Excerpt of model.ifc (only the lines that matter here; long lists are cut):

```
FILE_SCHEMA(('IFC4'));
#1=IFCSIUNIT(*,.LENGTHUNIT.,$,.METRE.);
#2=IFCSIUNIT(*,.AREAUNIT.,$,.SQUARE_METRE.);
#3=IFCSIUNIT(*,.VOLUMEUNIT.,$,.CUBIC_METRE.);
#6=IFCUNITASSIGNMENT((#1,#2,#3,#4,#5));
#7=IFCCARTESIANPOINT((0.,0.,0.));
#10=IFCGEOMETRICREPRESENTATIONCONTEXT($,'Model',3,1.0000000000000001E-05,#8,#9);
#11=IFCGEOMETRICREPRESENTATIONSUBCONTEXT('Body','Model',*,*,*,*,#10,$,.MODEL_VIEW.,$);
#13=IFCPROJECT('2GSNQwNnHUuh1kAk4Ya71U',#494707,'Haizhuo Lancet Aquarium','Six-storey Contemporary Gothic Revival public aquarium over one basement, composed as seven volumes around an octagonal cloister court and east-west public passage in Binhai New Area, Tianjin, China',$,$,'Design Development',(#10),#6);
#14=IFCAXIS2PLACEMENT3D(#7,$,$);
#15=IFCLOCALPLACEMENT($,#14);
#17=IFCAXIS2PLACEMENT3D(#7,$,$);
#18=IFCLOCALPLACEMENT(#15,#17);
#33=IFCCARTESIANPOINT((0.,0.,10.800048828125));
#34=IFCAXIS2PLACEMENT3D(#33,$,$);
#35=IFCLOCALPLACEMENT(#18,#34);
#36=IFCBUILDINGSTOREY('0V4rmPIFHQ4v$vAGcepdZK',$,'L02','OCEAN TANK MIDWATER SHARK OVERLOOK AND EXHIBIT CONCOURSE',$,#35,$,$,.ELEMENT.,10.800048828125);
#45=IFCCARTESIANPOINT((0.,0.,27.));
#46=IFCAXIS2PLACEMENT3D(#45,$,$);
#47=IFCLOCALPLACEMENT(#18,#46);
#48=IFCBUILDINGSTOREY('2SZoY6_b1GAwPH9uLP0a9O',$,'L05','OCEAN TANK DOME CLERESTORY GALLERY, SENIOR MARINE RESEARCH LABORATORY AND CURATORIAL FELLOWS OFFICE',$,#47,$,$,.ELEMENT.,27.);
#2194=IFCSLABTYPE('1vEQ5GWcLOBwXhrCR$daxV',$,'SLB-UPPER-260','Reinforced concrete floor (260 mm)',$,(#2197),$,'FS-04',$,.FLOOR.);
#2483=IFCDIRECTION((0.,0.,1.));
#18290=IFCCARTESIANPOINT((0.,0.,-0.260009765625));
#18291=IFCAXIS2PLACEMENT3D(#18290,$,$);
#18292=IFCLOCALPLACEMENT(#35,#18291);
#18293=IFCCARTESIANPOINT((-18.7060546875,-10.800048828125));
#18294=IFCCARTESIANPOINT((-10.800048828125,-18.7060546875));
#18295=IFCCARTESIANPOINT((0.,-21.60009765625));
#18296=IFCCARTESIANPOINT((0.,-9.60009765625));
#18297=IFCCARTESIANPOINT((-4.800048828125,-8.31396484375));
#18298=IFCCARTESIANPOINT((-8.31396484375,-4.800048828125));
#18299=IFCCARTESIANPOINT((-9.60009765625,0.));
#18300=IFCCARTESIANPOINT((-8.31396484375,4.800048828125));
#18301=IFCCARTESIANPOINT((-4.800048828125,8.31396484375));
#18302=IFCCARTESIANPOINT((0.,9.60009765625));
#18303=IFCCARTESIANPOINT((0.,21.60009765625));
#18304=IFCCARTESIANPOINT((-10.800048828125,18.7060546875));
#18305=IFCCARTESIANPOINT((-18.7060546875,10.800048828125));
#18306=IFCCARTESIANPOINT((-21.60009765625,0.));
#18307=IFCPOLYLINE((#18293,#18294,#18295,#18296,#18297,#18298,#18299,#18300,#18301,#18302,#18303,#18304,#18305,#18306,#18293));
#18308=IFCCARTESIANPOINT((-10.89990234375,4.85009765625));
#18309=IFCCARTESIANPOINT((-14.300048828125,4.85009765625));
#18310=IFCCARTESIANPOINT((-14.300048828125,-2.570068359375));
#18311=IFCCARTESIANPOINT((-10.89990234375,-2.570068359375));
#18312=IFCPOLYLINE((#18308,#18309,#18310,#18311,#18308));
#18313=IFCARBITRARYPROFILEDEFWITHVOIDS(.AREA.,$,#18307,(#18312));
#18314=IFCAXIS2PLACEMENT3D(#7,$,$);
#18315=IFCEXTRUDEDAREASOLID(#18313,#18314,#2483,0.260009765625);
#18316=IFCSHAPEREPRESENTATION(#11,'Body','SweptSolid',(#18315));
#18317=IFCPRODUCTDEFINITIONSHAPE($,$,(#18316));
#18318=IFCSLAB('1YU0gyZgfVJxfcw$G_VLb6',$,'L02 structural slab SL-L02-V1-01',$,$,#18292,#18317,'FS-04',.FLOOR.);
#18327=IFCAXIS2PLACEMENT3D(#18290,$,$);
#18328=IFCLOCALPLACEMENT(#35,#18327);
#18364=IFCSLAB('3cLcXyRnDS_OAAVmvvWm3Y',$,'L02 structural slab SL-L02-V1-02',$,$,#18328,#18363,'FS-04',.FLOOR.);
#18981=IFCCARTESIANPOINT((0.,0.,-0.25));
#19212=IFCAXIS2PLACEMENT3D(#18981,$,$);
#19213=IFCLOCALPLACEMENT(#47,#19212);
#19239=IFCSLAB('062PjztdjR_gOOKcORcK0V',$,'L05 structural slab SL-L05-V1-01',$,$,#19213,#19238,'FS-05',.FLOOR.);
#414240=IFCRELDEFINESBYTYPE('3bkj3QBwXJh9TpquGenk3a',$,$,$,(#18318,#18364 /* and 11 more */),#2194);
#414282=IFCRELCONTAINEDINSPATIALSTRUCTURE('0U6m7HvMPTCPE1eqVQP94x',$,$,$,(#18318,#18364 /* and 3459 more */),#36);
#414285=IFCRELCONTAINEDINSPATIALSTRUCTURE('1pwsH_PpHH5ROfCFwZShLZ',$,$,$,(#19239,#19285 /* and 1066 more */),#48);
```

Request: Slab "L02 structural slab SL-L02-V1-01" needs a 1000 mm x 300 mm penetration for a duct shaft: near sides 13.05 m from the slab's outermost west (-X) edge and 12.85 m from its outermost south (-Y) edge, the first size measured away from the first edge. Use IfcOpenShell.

```python
import numpy as np
import ifcopenshell
import ifcopenshell.api.feature
import ifcopenshell.api.geometry
import ifcopenshell.api.root
import ifcopenshell.geom
import ifcopenshell.util.placement
import ifcopenshell.util.representation
import ifcopenshell.util.shape
import ifcopenshell.util.unit

model = ifcopenshell.open("model.ifc")
unit_scale = ifcopenshell.util.unit.calculate_unit_scale(model)
settings = ifcopenshell.geom.settings()


def volume(element):
    """Net volume in cubic metres, openings subtracted."""
    shape = ifcopenshell.geom.create_shape(settings, element)
    return ifcopenshell.util.shape.get_volume(shape.geometry)


slab = model.by_id(18318)
before = volume(slab)

# Extent in the slab's own axes, in metres. The edges named are its -X and -Y sides.
slab_shape = ifcopenshell.geom.create_shape(settings, slab)
vertices = ifcopenshell.util.shape.get_vertices(slab_shape.geometry)
x_min, y_min, bottom = vertices.min(axis=0)
top = vertices[:, 2].max()

opening = ifcopenshell.api.root.create_entity(model, ifc_class="IfcOpeningElement", name="Duct shaft opening", predefined_type="OPENING")
context = ifcopenshell.util.representation.get_context(model, "Model", "Body", "MODEL_VIEW")
width, depth = 1, 0.3
outline = [(0.0, 0.0), (width, 0.0), (width, depth), (0.0, depth), (0.0, 0.0)]
# Overshoot both faces by 50 mm so the cut is clean.
shape = ifcopenshell.api.geometry.add_slab_representation(
    model, context=context, depth=top - bottom + 0.1, polyline=outline
)
ifcopenshell.api.geometry.assign_representation(model, product=opening, representation=shape)

matrix = ifcopenshell.util.placement.get_local_placement(slab.ObjectPlacement)
matrix[:, 3] = matrix @ np.append(np.array([x_min + 13.05, y_min + 12.85, bottom - 0.05]) / unit_scale, 1.0)
ifcopenshell.api.geometry.edit_object_placement(model, product=opening, matrix=matrix, is_si=False)
ifcopenshell.api.feature.add_feature(model, feature=opening, element=slab)

after = volume(slab)

print(f"slab volume {before:.3f} -> {after:.3f} m3")

model.write("model_rev.ifc")
```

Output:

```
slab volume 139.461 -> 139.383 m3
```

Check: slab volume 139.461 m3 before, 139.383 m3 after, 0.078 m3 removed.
